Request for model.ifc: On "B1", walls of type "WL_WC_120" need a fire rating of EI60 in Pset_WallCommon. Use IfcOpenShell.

First a look at what the model holds.

```python
import ifcopenshell
import ifcopenshell.util.element

model = ifcopenshell.open("model.ifc")
print(model.schema)
storey = next(s for s in model.by_type("IfcBuildingStorey") if s.Name == "B1")
walls = [e for e in ifcopenshell.util.element.get_decomposition(storey) if e.is_a("IfcWall")]
seen = {}
for e in walls:
    element_type = ifcopenshell.util.element.get_type(e)
    key = (element_type.Name if element_type != e and element_type else None, ifcopenshell.util.element.get_pset(e, "Pset_WallCommon", "FireRating"))
    seen[key] = seen.get(key, 0) + 1
for (name, value), count in sorted(seen.items(), key=str):
    print(count, "x", name, "|", value)
```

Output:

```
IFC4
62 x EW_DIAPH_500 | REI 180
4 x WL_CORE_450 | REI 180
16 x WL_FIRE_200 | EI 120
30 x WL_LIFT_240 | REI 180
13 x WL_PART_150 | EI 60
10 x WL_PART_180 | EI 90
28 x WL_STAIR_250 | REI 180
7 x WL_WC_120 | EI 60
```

```python
import ifcopenshell
import ifcopenshell.api.pset
import ifcopenshell.util.element

model = ifcopenshell.open("model.ifc")

storey = next(s for s in model.by_type("IfcBuildingStorey") if s.Name == "B1")
walls = [e for e in ifcopenshell.util.element.get_decomposition(storey) if e.is_a("IfcWall")]

count = 0
for e in walls:
    element_type = ifcopenshell.util.element.get_type(e)
    if element_type in (None, e) or element_type.Name != "WL_WC_120":
        continue
    # add_pset returns the element's existing set when there is one.
    pset = ifcopenshell.api.pset.add_pset(model, product=e, name="Pset_WallCommon")
    ifcopenshell.api.pset.edit_pset(model, pset=pset, properties={"FireRating": "EI60"})
    count += 1

print(count, "walls updated")

model.write("model_edited.ifc")
```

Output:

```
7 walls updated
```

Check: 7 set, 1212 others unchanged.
